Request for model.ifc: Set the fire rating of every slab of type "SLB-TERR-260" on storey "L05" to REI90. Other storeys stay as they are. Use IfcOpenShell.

First a look at what the model holds.

```python
import ifcopenshell
import ifcopenshell.util.element

model = ifcopenshell.open("model.ifc")
print(model.schema)
storey = next(s for s in model.by_type("IfcBuildingStorey") if s.Name == "L05")
slabs = [e for e in ifcopenshell.util.element.get_decomposition(storey) if e.is_a("IfcSlab")]
seen = {}
for e in slabs:
    element_type = ifcopenshell.util.element.get_type(e)
    key = (element_type.Name if element_type != e and element_type else None, ifcopenshell.util.element.get_pset(e, "Pset_SlabCommon", "FireRating"))
    seen[key] = seen.get(key, 0) + 1
for (name, value), count in sorted(seen.items(), key=str):
    print(count, "x", name, "|", value)
```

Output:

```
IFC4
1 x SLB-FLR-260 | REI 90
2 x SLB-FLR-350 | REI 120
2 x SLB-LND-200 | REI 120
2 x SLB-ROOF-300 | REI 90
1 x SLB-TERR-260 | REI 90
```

```python
import ifcopenshell
import ifcopenshell.api.pset
import ifcopenshell.util.element

model = ifcopenshell.open("model.ifc")

storey = next(s for s in model.by_type("IfcBuildingStorey") if s.Name == "L05")
slabs = [e for e in ifcopenshell.util.element.get_decomposition(storey) if e.is_a("IfcSlab")]

count = 0
for e in slabs:
    element_type = ifcopenshell.util.element.get_type(e)
    if element_type in (None, e) or element_type.Name != "SLB-TERR-260":
        continue
    # add_pset returns the element's existing set when there is one.
    pset = ifcopenshell.api.pset.add_pset(model, product=e, name="Pset_SlabCommon")
    ifcopenshell.api.pset.edit_pset(model, pset=pset, properties={"FireRating": "REI90"})
    count += 1

print(count, "slabs updated")

model.write("model-out.ifc")
```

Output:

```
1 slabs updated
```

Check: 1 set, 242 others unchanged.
